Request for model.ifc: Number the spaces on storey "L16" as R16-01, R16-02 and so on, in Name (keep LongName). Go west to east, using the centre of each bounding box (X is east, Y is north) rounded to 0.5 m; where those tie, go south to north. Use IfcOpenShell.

First a look at what the model holds.

```python
import ifcopenshell
import ifcopenshell.util.element
import ifcopenshell.util.placement

model = ifcopenshell.open("model.ifc")
print(model.schema)
storey = next(s for s in model.by_type("IfcBuildingStorey") if s.Name == "L16")
spaces = [e for e in ifcopenshell.util.element.get_decomposition(storey) if e.is_a("IfcSpace")]
for e in sorted(spaces, key=lambda e: e.id()):
    origin = ifcopenshell.util.placement.get_local_placement(e.ObjectPlacement)[:3, 3]
    print(e.id(), e.Name, e.LongName, origin.round(2) + 0.0, sep=" | ")
```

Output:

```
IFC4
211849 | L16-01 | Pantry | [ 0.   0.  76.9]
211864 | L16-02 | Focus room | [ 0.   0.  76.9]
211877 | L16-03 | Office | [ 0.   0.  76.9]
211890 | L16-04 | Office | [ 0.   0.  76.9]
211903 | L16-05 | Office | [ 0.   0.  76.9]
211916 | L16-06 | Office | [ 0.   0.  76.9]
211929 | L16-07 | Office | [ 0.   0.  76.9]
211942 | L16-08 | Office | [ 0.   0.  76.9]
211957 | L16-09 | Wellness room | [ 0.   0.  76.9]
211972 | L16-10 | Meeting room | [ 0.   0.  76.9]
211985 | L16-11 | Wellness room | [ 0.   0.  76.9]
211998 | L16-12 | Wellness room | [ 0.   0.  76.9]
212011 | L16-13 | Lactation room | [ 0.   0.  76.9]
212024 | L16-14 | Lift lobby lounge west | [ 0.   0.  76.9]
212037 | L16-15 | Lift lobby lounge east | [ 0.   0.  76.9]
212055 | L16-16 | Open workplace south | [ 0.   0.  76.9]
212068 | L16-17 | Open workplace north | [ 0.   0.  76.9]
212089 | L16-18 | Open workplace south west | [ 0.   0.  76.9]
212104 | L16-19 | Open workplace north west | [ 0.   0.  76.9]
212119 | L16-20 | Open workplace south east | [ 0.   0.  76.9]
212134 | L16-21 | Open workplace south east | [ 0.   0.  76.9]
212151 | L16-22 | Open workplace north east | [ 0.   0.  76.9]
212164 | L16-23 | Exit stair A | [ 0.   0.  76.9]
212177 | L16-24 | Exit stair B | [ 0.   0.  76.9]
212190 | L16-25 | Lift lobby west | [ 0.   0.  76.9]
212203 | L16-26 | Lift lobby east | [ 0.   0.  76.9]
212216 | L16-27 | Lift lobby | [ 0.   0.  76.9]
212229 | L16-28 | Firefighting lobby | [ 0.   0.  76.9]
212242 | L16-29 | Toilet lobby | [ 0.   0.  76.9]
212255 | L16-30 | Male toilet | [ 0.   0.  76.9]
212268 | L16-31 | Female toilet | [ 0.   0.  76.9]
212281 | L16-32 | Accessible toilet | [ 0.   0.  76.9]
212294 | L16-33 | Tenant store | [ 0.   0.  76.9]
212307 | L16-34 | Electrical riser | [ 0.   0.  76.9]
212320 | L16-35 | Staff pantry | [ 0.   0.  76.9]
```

```python
import ifcopenshell
import ifcopenshell.geom
import ifcopenshell.util.element
import ifcopenshell.util.shape

model = ifcopenshell.open("model.ifc")
settings = ifcopenshell.geom.settings()
settings.set("use-world-coords", True)


def centre(element):
    shape = ifcopenshell.geom.create_shape(settings, element)
    return ifcopenshell.util.shape.get_bbox_centroid(shape.geometry)


storey = next(s for s in model.by_type("IfcBuildingStorey") if s.Name == "L16")
spaces = [e for e in ifcopenshell.util.element.get_decomposition(storey) if e.is_a("IfcSpace")]

# Insertion points can sit at a corner or the storey origin, so sort by the geometry (in metres).
centres = {e: centre(e) for e in spaces}
spaces.sort(key=lambda e: (round(centres[e][0] / 0.5), centres[e][1]))

for i, e in enumerate(spaces, start=1):
    number = f"R16-{i:02d}"
    e.Name = number
    print(e.id(), number)

model.write("model_edited.ifc")
```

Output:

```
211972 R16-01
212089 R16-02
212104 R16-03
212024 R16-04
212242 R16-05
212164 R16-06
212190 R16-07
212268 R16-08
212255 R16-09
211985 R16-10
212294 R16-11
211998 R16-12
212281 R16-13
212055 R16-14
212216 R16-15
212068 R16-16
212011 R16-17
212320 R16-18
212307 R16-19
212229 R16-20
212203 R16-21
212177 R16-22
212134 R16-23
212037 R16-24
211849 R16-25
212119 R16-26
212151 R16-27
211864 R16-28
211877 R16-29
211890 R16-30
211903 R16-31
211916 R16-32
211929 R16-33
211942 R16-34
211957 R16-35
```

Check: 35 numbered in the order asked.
